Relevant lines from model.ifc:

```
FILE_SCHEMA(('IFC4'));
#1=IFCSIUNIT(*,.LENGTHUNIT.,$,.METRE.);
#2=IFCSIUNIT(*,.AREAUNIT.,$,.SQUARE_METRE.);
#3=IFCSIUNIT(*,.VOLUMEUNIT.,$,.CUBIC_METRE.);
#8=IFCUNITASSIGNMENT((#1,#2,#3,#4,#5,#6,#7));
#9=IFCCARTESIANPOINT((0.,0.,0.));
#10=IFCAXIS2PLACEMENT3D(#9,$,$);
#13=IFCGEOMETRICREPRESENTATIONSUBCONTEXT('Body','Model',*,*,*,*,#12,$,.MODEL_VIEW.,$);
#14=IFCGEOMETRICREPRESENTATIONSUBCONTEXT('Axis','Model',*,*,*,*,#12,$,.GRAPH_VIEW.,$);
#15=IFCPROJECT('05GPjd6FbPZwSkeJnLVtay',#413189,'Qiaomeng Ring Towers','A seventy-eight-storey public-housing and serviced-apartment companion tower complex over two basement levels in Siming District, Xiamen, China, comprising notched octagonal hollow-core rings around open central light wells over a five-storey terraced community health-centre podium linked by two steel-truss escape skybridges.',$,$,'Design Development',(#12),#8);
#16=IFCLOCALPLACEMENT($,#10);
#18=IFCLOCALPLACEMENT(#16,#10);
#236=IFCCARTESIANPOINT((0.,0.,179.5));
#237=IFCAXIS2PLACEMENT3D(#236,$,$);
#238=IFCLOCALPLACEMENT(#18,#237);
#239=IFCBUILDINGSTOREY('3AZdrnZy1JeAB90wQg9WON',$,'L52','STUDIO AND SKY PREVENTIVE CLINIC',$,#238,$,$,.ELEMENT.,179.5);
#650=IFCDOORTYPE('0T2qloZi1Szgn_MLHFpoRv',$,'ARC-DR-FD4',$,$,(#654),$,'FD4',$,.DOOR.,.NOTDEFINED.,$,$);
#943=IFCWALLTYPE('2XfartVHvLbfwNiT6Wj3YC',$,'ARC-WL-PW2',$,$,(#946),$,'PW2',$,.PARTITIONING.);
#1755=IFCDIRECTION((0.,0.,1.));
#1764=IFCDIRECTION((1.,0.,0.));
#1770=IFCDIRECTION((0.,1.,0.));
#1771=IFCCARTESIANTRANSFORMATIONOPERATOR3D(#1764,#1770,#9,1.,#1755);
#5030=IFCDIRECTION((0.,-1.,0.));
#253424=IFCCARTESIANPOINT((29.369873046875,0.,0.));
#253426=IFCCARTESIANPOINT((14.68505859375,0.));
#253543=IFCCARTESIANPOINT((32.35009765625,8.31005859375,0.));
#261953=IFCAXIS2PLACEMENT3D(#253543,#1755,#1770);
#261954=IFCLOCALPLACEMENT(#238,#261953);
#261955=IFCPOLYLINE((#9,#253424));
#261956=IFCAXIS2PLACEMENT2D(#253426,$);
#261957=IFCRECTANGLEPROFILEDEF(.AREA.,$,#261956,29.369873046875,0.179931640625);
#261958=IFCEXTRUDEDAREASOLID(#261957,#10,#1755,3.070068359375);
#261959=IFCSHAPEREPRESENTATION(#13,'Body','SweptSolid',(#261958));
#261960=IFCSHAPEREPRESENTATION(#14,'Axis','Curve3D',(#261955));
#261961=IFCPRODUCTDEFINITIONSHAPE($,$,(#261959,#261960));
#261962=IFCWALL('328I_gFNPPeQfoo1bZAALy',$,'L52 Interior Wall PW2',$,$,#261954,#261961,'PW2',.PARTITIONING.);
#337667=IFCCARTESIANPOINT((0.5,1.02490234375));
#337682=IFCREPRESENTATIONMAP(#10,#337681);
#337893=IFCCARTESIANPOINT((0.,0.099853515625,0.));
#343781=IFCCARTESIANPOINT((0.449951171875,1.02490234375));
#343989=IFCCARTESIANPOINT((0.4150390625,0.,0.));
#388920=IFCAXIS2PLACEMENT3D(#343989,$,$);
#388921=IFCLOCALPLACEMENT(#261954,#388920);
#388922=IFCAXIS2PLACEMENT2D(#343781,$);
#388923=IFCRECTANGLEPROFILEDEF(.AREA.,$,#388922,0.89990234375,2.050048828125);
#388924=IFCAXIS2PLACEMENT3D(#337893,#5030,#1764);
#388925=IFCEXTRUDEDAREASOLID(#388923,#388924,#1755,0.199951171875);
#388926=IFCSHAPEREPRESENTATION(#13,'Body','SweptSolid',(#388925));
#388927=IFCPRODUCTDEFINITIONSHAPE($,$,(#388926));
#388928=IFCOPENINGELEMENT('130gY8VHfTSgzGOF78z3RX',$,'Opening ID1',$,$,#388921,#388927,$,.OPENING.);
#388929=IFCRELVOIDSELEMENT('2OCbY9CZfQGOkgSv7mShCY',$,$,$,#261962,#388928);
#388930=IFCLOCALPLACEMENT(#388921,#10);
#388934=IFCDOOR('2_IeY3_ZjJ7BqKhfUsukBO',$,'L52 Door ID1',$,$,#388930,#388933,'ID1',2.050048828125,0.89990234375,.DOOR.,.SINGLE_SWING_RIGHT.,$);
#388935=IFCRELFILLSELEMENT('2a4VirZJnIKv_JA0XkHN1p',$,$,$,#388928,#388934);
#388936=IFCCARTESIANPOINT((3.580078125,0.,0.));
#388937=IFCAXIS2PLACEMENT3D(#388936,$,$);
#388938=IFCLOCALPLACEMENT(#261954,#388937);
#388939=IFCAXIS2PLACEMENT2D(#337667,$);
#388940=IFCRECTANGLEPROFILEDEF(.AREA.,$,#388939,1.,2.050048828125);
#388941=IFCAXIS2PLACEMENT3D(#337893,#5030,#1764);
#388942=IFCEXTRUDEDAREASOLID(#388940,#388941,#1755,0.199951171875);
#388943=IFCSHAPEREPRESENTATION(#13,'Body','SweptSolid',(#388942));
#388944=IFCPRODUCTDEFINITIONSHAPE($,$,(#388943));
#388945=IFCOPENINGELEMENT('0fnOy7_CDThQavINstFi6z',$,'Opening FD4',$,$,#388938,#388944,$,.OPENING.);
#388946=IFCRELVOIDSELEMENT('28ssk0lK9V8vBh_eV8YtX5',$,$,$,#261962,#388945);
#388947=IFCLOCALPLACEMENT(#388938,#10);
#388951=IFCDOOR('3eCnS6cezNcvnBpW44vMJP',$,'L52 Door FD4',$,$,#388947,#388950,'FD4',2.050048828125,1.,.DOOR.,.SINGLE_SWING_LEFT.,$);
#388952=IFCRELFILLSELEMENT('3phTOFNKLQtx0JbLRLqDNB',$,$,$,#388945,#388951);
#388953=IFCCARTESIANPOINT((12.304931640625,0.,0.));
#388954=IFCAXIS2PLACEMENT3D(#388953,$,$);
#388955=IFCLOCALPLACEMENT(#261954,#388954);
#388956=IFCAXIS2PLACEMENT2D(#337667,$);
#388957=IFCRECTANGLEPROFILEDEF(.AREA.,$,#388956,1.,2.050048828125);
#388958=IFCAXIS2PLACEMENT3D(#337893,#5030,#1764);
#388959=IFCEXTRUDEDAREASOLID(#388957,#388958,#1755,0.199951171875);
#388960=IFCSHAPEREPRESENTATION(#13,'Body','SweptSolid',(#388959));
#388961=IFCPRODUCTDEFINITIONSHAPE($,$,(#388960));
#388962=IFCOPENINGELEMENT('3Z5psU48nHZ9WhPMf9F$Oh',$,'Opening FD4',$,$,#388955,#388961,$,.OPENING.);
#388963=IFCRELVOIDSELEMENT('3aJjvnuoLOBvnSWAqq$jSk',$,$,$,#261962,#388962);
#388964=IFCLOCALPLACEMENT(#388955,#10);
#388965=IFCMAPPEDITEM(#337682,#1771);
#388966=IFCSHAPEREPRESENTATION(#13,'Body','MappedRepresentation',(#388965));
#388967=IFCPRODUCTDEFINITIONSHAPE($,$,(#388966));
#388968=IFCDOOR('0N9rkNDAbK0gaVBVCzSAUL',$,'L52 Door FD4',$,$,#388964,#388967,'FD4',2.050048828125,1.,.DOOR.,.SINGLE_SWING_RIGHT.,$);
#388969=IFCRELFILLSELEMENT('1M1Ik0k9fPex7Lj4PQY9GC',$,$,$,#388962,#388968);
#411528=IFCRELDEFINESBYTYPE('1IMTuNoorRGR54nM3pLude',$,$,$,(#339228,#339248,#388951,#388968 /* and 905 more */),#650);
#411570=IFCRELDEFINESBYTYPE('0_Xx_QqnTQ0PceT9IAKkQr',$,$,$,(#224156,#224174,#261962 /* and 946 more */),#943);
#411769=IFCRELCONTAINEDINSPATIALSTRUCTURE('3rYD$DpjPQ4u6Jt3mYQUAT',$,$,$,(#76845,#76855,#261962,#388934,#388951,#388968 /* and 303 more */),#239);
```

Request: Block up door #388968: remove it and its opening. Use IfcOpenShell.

```python
import ifcopenshell
import ifcopenshell.api.feature
import ifcopenshell.api.root
import ifcopenshell.geom
import ifcopenshell.util.shape

model = ifcopenshell.open("model.ifc")
settings = ifcopenshell.geom.settings()


def volume(element):
    """Net volume in cubic metres, openings subtracted."""
    shape = ifcopenshell.geom.create_shape(settings, element)
    return ifcopenshell.util.shape.get_volume(shape.geometry)


door = model.by_guid("0N9rkNDAbK0gaVBVCzSAUL")
opening = door.FillsVoids[0].RelatingOpeningElement
wall = opening.VoidsElements[0].RelatingBuildingElement
before = volume(wall)

ifcopenshell.api.root.remove_product(model, product=door)
ifcopenshell.api.feature.remove_feature(model, feature=opening)

after = volume(wall)

print(f"wall volume {before:.3f} -> {after:.3f} m3")

model.write("model_edited.ifc")
```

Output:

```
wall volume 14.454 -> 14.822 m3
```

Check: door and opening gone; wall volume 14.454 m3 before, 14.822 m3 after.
